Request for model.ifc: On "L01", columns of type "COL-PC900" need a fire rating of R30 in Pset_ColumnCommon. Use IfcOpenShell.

First a look at what the model holds.

```python
import ifcopenshell
import ifcopenshell.util.element

model = ifcopenshell.open("model.ifc")
print(model.schema)
storey = next(s for s in model.by_type("IfcBuildingStorey") if s.Name == "L01")
columns = [e for e in ifcopenshell.util.element.get_decomposition(storey) if e.is_a("IfcColumn")]
seen = {}
for e in columns:
    element_type = ifcopenshell.util.element.get_type(e)
    key = (element_type.Name if element_type != e and element_type else None, ifcopenshell.util.element.get_pset(e, "Pset_ColumnCommon", "FireRating"))
    seen[key] = seen.get(key, 0) + 1
for (name, value), count in sorted(seen.items(), key=str):
    print(count, "x", name, "|", value)
```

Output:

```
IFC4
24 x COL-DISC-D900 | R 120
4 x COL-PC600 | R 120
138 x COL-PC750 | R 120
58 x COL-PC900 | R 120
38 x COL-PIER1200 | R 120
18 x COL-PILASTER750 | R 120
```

```python
import ifcopenshell
import ifcopenshell.api.pset
import ifcopenshell.util.element

model = ifcopenshell.open("model.ifc")

storey = next(s for s in model.by_type("IfcBuildingStorey") if s.Name == "L01")
columns = [e for e in ifcopenshell.util.element.get_decomposition(storey) if e.is_a("IfcColumn")]

count = 0
for e in columns:
    element_type = ifcopenshell.util.element.get_type(e)
    if element_type in (None, e) or element_type.Name != "COL-PC900":
        continue
    # add_pset returns the element's existing set when there is one.
    pset = ifcopenshell.api.pset.add_pset(model, product=e, name="Pset_ColumnCommon")
    ifcopenshell.api.pset.edit_pset(model, pset=pset, properties={"FireRating": "R30"})
    count += 1

print(count, "columns updated")

model.write("model-out.ifc")
```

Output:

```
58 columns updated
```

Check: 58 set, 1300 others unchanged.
